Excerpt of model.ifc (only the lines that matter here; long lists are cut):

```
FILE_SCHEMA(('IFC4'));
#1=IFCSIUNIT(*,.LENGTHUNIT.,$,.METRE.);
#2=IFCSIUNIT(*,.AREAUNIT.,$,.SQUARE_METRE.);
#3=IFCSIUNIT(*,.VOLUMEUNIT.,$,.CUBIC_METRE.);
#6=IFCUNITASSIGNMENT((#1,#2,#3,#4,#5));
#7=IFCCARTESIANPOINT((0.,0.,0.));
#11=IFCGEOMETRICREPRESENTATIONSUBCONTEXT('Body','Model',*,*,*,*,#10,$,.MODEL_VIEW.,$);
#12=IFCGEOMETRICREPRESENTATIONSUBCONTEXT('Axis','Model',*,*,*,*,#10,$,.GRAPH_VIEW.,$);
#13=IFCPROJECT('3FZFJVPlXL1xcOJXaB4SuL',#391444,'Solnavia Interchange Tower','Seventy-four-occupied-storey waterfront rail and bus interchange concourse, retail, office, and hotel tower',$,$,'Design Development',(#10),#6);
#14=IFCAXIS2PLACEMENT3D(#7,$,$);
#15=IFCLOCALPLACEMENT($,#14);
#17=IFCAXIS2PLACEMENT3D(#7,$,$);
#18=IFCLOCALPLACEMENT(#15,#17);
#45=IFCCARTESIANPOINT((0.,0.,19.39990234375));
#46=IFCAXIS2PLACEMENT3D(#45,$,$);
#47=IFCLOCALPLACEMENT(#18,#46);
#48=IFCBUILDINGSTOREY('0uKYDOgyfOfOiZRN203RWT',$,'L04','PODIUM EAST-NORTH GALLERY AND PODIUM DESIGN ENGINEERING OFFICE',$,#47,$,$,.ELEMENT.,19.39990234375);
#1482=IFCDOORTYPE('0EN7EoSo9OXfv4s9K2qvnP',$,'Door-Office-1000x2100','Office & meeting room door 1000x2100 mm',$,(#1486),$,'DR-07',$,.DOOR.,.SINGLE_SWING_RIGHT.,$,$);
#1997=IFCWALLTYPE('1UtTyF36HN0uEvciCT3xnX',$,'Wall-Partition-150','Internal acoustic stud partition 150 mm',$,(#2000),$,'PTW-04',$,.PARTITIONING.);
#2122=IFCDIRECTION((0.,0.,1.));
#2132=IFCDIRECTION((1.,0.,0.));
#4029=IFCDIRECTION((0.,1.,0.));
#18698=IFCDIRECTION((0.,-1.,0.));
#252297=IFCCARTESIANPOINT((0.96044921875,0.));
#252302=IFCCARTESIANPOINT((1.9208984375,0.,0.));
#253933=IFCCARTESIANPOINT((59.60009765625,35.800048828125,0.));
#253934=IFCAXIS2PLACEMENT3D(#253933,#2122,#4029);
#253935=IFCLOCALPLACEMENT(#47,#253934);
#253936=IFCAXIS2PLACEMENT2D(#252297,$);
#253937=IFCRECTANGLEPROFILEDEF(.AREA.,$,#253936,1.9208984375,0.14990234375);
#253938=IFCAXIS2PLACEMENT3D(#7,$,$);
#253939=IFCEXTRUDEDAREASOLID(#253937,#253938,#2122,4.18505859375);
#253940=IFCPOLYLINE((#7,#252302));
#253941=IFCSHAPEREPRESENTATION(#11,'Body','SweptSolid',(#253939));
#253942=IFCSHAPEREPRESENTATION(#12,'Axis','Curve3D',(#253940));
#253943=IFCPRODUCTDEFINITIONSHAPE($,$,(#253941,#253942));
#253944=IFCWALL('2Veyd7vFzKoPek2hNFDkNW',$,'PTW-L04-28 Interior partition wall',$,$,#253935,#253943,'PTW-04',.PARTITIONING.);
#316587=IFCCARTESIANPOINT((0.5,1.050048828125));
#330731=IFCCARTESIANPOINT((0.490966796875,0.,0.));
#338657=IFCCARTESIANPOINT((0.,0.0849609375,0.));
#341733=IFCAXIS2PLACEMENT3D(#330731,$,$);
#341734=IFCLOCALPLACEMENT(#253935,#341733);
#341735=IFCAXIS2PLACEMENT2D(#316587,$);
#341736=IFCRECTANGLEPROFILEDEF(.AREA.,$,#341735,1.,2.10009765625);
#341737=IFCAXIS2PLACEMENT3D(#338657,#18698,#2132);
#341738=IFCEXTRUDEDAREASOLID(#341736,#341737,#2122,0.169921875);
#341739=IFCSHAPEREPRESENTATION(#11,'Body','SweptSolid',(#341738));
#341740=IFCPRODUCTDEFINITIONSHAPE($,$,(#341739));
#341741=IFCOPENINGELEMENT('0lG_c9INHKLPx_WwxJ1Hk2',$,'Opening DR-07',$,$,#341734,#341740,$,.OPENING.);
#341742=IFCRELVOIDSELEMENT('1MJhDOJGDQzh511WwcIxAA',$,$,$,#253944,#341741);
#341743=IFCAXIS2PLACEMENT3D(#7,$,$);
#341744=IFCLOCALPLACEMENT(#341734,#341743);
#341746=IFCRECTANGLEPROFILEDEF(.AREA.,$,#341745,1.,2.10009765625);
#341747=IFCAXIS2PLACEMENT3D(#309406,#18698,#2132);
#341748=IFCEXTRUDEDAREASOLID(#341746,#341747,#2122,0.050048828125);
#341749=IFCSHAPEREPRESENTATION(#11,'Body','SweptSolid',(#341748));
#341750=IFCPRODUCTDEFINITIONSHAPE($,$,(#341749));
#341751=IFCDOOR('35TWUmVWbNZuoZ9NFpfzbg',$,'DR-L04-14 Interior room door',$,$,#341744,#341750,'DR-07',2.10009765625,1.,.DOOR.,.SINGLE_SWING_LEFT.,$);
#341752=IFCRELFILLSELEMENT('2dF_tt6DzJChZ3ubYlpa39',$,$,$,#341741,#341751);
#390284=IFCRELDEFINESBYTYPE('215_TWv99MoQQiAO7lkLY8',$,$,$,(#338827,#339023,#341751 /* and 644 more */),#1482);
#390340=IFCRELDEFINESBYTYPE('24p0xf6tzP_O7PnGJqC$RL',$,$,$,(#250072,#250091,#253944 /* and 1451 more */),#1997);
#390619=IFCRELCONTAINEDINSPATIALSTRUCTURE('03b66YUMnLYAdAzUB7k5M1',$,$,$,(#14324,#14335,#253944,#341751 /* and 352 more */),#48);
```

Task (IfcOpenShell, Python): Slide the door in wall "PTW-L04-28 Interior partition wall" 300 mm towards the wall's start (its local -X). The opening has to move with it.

```python
import ifcopenshell
import ifcopenshell.api.geometry
import ifcopenshell.util.placement

model = ifcopenshell.open("model.ifc")

door = model.by_guid("35TWUmVWbNZuoZ9NFpfzbg")
opening = door.FillsVoids[0].RelatingOpeningElement
wall = opening.VoidsElements[0].RelatingBuildingElement

wall_matrix = ifcopenshell.util.placement.get_local_placement(wall.ObjectPlacement)
shift = wall_matrix[:3, 0] * -0.3
before = ifcopenshell.util.placement.get_local_placement(door.ObjectPlacement)[:3, 3].copy()

# The door is placed relative to its opening, so it follows when the opening moves.
matrix = ifcopenshell.util.placement.get_local_placement(opening.ObjectPlacement)
matrix[:3, 3] += shift
ifcopenshell.api.geometry.edit_object_placement(
    model, product=opening, matrix=matrix, is_si=False, should_transform_children=True
)

after = ifcopenshell.util.placement.get_local_placement(door.ObjectPlacement)[:3, 3]
print("door moved by", (after - before).round(3) + 0.0)

model.write("model_updated.ifc")
```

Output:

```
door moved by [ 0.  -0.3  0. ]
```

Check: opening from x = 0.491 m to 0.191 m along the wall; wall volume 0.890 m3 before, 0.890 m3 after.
